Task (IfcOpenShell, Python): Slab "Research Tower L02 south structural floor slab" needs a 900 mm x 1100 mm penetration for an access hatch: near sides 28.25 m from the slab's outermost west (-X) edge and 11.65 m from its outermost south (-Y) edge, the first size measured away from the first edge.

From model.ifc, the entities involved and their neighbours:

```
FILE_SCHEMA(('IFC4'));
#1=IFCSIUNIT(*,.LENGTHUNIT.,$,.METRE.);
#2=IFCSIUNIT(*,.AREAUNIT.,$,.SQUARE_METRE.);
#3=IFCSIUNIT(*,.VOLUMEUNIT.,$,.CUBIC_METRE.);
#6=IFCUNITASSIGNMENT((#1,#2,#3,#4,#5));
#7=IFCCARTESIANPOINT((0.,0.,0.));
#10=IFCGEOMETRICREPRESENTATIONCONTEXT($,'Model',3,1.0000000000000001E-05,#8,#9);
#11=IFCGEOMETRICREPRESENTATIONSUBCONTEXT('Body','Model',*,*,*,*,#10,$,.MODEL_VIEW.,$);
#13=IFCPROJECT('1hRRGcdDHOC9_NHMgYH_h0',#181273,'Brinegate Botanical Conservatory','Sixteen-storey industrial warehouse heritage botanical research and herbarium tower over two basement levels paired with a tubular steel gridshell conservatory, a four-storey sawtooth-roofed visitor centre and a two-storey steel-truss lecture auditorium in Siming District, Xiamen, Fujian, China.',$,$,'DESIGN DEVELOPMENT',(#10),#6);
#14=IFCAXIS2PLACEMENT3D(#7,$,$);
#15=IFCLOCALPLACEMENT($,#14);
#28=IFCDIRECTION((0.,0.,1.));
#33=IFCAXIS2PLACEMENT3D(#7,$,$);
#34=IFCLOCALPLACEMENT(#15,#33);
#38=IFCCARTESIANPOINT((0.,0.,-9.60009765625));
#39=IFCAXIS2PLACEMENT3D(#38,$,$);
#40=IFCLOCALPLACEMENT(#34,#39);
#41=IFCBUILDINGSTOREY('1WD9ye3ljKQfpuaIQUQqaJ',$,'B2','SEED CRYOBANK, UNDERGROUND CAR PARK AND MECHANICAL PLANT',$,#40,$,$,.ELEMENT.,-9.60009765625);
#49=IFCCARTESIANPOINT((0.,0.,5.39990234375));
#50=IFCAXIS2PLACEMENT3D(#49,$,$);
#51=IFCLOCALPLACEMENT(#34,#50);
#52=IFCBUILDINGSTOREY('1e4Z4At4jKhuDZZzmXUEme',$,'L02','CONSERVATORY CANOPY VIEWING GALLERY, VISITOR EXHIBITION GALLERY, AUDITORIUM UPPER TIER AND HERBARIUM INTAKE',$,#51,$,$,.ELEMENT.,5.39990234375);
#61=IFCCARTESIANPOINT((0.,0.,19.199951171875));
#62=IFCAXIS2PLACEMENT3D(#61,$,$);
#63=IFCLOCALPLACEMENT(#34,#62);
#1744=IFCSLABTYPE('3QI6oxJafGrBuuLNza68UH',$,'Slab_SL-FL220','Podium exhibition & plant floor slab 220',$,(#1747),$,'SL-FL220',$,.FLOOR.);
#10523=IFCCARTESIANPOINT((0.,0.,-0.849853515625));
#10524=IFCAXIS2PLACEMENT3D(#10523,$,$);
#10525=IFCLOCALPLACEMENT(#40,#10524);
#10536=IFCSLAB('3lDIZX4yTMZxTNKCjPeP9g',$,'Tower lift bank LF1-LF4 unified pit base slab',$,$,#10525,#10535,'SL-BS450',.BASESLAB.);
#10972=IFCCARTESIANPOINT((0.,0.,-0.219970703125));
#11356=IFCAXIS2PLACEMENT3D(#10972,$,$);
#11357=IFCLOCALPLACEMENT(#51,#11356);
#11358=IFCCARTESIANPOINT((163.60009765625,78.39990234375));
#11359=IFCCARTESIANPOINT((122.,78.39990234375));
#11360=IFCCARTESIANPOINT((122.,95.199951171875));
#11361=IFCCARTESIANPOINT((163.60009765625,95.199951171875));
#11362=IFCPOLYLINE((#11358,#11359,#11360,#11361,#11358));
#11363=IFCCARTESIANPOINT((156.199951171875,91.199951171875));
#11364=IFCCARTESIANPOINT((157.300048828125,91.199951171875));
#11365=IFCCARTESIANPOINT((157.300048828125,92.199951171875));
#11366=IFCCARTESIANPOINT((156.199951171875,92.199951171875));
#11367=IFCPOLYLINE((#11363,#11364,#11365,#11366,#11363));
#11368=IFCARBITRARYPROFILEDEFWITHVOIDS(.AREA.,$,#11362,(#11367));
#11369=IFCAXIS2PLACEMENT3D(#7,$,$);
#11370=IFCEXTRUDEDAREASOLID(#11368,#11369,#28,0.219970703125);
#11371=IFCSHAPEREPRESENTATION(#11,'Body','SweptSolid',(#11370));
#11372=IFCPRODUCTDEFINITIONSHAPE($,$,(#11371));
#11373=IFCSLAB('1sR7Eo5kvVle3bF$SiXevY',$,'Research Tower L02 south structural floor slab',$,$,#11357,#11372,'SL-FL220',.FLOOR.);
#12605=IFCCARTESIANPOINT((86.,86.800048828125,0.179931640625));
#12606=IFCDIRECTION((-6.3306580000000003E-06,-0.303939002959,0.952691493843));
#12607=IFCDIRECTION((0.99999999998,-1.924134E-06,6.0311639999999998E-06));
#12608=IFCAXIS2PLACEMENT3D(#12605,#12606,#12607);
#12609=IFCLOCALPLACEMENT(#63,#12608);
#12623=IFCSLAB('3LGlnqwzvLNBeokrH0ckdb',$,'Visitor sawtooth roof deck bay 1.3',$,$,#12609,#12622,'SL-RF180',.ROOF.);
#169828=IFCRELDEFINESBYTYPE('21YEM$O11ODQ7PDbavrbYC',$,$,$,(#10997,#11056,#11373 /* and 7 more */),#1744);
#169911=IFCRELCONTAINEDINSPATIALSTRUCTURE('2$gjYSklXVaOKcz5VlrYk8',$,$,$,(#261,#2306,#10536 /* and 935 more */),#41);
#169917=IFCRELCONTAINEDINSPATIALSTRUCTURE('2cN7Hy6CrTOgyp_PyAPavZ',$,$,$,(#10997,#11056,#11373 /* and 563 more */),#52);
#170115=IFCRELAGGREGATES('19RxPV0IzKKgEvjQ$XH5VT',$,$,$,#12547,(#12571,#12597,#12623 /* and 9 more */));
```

```python
import numpy as np
import ifcopenshell
import ifcopenshell.api.feature
import ifcopenshell.api.geometry
import ifcopenshell.api.root
import ifcopenshell.geom
import ifcopenshell.util.placement
import ifcopenshell.util.representation
import ifcopenshell.util.shape
import ifcopenshell.util.unit

model = ifcopenshell.open("model.ifc")
unit_scale = ifcopenshell.util.unit.calculate_unit_scale(model)
settings = ifcopenshell.geom.settings()


def volume(element):
    """Net volume in cubic metres, openings subtracted."""
    shape = ifcopenshell.geom.create_shape(settings, element)
    return ifcopenshell.util.shape.get_volume(shape.geometry)


slab = model.by_guid("1sR7Eo5kvVle3bF$SiXevY")
before = volume(slab)

# Extent in the slab's own axes, in metres. The edges named are its -X and -Y sides.
slab_shape = ifcopenshell.geom.create_shape(settings, slab)
vertices = ifcopenshell.util.shape.get_vertices(slab_shape.geometry)
x_min, y_min, bottom = vertices.min(axis=0)
top = vertices[:, 2].max()

opening = ifcopenshell.api.root.create_entity(model, ifc_class="IfcOpeningElement", name="Access hatch opening", predefined_type="OPENING")
context = ifcopenshell.util.representation.get_context(model, "Model", "Body", "MODEL_VIEW")
width, depth = 0.9, 1.1
outline = [(0.0, 0.0), (width, 0.0), (width, depth), (0.0, depth), (0.0, 0.0)]
# Overshoot both faces by 50 mm so the cut is clean.
shape = ifcopenshell.api.geometry.add_slab_representation(
    model, context=context, depth=top - bottom + 0.1, polyline=outline
)
ifcopenshell.api.geometry.assign_representation(model, product=opening, representation=shape)

matrix = ifcopenshell.util.placement.get_local_placement(slab.ObjectPlacement)
matrix[:, 3] = matrix @ np.append(np.array([x_min + 28.25, y_min + 11.65, bottom - 0.05]) / unit_scale, 1.0)
ifcopenshell.api.geometry.edit_object_placement(model, product=opening, matrix=matrix, is_si=False)
ifcopenshell.api.feature.add_feature(model, feature=opening, element=slab)

after = volume(slab)

print(f"slab volume {before:.3f} -> {after:.3f} m3")

model.write("model_rev.ifc")
```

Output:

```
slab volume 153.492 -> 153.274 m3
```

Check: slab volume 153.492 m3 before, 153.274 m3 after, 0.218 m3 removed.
